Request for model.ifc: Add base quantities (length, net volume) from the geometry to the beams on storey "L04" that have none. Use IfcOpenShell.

First a look at what the model holds.

```python
import ifcopenshell
import ifcopenshell.util.element
import ifcopenshell.util.unit

model = ifcopenshell.open("model.ifc")
print(model.schema)
for unit_type in ("LENGTHUNIT", "AREAUNIT", "VOLUMEUNIT"):
    print(unit_type, ifcopenshell.util.unit.calculate_unit_scale(model, unit_type))
storey = next(s for s in model.by_type("IfcBuildingStorey") if s.Name == "L04")
beams = [e for e in ifcopenshell.util.element.get_decomposition(storey) if e.is_a("IfcBeam")]
for e in sorted(beams, key=lambda e: e.id()):
    print(e.id(), e.is_a(), e.Name, list(ifcopenshell.util.element.get_psets(e, qtos_only=True)), sep=" | ")
```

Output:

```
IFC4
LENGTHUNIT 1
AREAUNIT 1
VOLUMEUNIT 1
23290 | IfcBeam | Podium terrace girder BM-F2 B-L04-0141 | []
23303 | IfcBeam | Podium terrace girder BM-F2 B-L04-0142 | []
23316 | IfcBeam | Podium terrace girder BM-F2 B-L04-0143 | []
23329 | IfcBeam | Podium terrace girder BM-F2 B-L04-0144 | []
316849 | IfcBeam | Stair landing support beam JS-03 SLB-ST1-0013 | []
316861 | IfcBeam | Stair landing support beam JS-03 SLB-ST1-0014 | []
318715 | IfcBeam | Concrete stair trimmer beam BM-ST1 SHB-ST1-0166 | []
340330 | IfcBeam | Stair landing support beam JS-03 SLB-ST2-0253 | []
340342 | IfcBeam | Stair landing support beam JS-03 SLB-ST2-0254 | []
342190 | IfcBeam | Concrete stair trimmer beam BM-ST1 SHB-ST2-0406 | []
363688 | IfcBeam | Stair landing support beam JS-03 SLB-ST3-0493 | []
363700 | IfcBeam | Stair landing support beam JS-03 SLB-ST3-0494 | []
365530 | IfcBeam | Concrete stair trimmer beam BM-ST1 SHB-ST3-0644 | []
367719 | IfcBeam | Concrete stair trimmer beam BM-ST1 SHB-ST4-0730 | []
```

```python
import ifcopenshell
import ifcopenshell.api.pset
import ifcopenshell.geom
import ifcopenshell.util.element
import ifcopenshell.util.shape
import ifcopenshell.util.unit

model = ifcopenshell.open("model.ifc")
unit_scale = ifcopenshell.util.unit.calculate_unit_scale(model)
volume_scale = ifcopenshell.util.unit.calculate_unit_scale(model, "VOLUMEUNIT")
settings = ifcopenshell.geom.settings()

storey = next(s for s in model.by_type("IfcBuildingStorey") if s.Name == "L04")
beams = [e for e in ifcopenshell.util.element.get_decomposition(storey) if e.is_a("IfcBeam")]

for e in sorted(beams, key=lambda e: e.id()):
    if ifcopenshell.util.element.get_psets(e, qtos_only=True, should_inherit=False):
        continue
    # Geometry comes back in metres, in the element's own axes.
    shape = ifcopenshell.geom.create_shape(settings, e)
    values = {
        "Length": ifcopenshell.util.shape.get_max_xyz(shape.geometry) / unit_scale,
        "NetVolume": ifcopenshell.util.shape.get_volume(shape.geometry) / volume_scale,
    }
    qto = ifcopenshell.api.pset.add_qto(model, product=e, name="Qto_BeamBaseQuantities")
    ifcopenshell.api.pset.edit_qto(model, qto=qto, properties=values)
    print(e.id(), {k: round(v, 3) for k, v in values.items()})

model.write("model_rev.ifc")
```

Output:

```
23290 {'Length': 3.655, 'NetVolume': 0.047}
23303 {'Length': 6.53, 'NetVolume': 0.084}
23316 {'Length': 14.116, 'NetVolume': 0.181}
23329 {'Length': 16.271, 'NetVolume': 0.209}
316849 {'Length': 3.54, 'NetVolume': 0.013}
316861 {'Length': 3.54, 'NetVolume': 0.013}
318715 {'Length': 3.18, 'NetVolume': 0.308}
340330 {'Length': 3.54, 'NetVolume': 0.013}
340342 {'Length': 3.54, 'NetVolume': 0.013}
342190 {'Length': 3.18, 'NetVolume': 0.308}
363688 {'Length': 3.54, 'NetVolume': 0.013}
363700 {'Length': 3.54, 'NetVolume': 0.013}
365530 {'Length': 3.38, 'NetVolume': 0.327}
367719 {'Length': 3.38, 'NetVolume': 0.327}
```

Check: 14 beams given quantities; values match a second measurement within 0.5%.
